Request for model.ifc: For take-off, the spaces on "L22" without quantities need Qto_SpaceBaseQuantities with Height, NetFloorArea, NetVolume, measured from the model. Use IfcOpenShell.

First a look at what the model holds.

```python
import ifcopenshell
import ifcopenshell.util.element
import ifcopenshell.util.unit

model = ifcopenshell.open("model.ifc")
print(model.schema)
for unit_type in ("LENGTHUNIT", "AREAUNIT", "VOLUMEUNIT"):
    print(unit_type, ifcopenshell.util.unit.calculate_unit_scale(model, unit_type))
storey = next(s for s in model.by_type("IfcBuildingStorey") if s.Name == "L22")
spaces = [e for e in ifcopenshell.util.element.get_decomposition(storey) if e.is_a("IfcSpace")]
for e in sorted(spaces, key=lambda e: e.id()):
    print(e.id(), e.is_a(), e.Name, list(ifcopenshell.util.element.get_psets(e, qtos_only=True)), sep=" | ")
```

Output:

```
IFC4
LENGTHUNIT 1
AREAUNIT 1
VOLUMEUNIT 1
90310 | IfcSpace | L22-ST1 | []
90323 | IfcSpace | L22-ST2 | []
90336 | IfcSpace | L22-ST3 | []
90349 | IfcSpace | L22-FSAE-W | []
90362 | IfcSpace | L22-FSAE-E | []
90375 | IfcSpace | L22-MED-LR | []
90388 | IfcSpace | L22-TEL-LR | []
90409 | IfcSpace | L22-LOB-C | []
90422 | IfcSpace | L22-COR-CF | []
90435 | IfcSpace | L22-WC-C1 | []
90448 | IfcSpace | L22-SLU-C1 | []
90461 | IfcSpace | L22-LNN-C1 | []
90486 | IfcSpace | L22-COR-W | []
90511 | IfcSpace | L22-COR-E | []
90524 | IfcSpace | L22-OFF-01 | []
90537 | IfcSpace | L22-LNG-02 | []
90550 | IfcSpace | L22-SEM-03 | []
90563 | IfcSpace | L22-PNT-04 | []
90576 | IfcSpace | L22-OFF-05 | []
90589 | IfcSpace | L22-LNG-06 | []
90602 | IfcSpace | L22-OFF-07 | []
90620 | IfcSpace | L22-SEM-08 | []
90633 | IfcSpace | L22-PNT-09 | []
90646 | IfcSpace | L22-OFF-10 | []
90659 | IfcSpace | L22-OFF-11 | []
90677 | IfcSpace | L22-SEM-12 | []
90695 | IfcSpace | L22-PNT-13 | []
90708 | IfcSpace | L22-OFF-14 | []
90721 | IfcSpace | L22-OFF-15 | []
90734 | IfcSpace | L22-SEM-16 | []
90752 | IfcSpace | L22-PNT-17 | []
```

```python
import ifcopenshell
import ifcopenshell.api.pset
import ifcopenshell.geom
import ifcopenshell.util.element
import ifcopenshell.util.shape
import ifcopenshell.util.unit

model = ifcopenshell.open("model.ifc")
unit_scale = ifcopenshell.util.unit.calculate_unit_scale(model)
area_scale = ifcopenshell.util.unit.calculate_unit_scale(model, "AREAUNIT")
volume_scale = ifcopenshell.util.unit.calculate_unit_scale(model, "VOLUMEUNIT")
settings = ifcopenshell.geom.settings()

storey = next(s for s in model.by_type("IfcBuildingStorey") if s.Name == "L22")
spaces = [e for e in ifcopenshell.util.element.get_decomposition(storey) if e.is_a("IfcSpace")]

for e in sorted(spaces, key=lambda e: e.id()):
    if ifcopenshell.util.element.get_psets(e, qtos_only=True, should_inherit=False):
        continue
    # Geometry comes back in metres, in the element's own axes.
    shape = ifcopenshell.geom.create_shape(settings, e)
    values = {
        "Height": ifcopenshell.util.shape.get_z(shape.geometry) / unit_scale,
        "NetFloorArea": ifcopenshell.util.shape.get_footprint_area(shape.geometry) / area_scale,
        "NetVolume": ifcopenshell.util.shape.get_volume(shape.geometry) / volume_scale,
    }
    qto = ifcopenshell.api.pset.add_qto(model, product=e, name="Qto_SpaceBaseQuantities")
    ifcopenshell.api.pset.edit_qto(model, qto=qto, properties=values)
    print(e.id(), {k: round(v, 3) for k, v in values.items()})

model.write("model_v2.ifc")
```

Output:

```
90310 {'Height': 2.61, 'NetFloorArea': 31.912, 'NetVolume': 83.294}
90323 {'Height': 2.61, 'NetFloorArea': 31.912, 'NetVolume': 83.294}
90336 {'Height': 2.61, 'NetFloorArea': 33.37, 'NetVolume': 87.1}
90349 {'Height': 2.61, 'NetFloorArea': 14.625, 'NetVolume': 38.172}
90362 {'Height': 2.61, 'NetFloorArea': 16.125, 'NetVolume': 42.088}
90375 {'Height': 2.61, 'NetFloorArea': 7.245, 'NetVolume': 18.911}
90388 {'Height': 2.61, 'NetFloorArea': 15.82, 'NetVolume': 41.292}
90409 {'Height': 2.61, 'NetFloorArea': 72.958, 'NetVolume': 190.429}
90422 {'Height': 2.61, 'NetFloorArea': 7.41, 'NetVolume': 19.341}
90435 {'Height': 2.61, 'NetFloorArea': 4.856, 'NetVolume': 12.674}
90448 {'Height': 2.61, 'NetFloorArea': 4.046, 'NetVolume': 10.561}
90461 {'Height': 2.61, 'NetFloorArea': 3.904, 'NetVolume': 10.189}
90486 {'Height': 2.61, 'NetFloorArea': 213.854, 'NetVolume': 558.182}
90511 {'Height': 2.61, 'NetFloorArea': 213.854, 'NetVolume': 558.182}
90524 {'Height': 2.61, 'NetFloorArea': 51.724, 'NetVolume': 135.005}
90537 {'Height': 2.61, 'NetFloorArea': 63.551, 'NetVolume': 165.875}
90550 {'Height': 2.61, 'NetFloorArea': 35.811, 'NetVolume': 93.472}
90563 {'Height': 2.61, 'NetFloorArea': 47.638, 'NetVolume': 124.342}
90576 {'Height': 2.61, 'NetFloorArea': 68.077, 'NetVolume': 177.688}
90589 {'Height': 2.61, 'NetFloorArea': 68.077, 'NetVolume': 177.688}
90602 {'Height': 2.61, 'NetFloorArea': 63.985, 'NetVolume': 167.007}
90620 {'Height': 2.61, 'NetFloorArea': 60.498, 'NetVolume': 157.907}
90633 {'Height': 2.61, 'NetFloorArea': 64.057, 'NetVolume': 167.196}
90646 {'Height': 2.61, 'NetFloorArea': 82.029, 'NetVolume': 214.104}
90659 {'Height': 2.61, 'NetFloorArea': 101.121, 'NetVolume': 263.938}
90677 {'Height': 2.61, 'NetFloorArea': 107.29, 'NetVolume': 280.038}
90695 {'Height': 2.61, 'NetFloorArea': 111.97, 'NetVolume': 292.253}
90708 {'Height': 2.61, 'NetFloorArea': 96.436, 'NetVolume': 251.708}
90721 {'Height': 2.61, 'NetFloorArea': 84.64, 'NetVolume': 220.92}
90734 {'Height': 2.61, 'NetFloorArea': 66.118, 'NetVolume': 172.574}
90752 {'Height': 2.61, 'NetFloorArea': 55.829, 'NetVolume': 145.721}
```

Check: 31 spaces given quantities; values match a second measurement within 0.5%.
